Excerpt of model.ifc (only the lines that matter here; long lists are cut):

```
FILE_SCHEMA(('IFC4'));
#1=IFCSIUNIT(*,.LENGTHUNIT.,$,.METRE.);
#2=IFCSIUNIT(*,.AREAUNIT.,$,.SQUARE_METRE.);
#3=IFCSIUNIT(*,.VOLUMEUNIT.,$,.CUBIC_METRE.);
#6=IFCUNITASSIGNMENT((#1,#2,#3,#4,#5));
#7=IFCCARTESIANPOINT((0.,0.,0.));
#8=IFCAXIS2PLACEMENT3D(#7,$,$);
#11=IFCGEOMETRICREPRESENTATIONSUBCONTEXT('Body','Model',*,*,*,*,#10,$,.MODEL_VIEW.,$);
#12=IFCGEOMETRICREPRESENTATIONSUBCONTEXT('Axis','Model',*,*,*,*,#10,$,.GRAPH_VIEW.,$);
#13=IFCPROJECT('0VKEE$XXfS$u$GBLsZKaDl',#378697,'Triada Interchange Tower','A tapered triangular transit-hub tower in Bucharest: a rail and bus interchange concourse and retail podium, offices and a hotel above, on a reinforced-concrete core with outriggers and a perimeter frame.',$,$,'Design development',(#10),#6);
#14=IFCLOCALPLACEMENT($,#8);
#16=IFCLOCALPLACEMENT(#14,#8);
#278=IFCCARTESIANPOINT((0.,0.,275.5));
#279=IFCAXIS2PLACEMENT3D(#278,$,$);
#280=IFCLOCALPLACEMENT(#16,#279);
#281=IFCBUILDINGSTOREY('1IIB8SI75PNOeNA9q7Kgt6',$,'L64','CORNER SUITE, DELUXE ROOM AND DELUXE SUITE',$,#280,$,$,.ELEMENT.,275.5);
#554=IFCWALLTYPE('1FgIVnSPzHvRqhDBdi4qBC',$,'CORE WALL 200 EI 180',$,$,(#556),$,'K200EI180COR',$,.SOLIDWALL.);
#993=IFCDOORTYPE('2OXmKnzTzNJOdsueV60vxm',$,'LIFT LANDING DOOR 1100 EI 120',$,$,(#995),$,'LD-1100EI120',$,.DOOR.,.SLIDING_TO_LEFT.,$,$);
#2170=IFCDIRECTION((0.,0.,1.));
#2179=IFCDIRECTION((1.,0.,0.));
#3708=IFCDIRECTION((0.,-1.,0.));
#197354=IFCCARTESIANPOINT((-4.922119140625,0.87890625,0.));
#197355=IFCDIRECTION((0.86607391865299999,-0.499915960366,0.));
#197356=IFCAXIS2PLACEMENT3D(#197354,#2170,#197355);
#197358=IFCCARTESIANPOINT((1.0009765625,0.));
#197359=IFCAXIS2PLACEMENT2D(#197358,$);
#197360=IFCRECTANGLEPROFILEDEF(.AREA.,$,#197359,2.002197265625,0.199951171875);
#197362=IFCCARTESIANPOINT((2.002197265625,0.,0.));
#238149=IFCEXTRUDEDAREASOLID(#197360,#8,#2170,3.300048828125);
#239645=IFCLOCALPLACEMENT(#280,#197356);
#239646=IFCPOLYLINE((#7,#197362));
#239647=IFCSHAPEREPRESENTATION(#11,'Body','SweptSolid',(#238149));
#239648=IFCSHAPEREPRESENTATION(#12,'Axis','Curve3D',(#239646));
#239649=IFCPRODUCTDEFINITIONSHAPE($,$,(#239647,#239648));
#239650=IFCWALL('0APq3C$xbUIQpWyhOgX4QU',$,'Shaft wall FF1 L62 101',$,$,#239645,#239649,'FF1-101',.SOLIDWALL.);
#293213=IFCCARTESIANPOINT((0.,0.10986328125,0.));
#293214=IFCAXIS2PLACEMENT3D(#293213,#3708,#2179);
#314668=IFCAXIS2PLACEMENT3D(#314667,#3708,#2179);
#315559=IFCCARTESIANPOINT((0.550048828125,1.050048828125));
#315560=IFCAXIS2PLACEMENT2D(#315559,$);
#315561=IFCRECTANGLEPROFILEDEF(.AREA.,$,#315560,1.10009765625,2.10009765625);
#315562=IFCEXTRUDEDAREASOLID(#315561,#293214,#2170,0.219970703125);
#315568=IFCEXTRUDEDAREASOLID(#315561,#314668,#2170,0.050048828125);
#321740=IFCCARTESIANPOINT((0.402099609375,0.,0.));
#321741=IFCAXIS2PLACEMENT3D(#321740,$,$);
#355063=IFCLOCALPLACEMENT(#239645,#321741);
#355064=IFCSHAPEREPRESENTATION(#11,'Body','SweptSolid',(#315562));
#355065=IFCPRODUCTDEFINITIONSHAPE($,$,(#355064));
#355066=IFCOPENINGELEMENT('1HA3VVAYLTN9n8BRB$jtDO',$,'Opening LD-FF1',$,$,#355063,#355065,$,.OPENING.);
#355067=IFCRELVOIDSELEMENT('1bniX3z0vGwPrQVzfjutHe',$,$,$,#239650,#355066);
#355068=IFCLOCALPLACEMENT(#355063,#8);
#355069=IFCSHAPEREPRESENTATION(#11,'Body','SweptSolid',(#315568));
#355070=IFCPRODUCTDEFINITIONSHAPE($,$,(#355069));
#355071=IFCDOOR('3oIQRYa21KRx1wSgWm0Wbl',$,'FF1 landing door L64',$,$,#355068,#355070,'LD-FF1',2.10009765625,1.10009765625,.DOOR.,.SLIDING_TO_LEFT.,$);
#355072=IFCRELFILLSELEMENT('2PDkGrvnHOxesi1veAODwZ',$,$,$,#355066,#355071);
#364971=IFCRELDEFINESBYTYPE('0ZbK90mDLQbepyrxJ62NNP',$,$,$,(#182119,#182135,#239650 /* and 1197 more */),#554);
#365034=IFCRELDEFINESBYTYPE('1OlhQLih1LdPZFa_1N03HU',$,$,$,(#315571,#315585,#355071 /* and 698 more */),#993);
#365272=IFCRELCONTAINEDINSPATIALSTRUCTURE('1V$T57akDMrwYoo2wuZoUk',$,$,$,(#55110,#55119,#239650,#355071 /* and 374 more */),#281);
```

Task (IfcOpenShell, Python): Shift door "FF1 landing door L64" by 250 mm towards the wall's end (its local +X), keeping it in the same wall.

```python
import ifcopenshell
import ifcopenshell.api.geometry
import ifcopenshell.util.placement
import ifcopenshell.util.unit

model = ifcopenshell.open("model.ifc")
unit_scale = ifcopenshell.util.unit.calculate_unit_scale(model)

door = model.by_id(355071)
opening = door.FillsVoids[0].RelatingOpeningElement
wall = opening.VoidsElements[0].RelatingBuildingElement

wall_matrix = ifcopenshell.util.placement.get_local_placement(wall.ObjectPlacement)
shift = wall_matrix[:3, 0] * 0.25 / unit_scale
before = ifcopenshell.util.placement.get_local_placement(door.ObjectPlacement)[:3, 3].copy()

# The door is placed relative to its opening, so it follows when the opening moves.
matrix = ifcopenshell.util.placement.get_local_placement(opening.ObjectPlacement)
matrix[:3, 3] += shift
ifcopenshell.api.geometry.edit_object_placement(
    model, product=opening, matrix=matrix, is_si=False, should_transform_children=True
)

after = ifcopenshell.util.placement.get_local_placement(door.ObjectPlacement)[:3, 3]
print("door moved by", (after - before).round(3) + 0.0)

model.write("model_rev.ifc")
```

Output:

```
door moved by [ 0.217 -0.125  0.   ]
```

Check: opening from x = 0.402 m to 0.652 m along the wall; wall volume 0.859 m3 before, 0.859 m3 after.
